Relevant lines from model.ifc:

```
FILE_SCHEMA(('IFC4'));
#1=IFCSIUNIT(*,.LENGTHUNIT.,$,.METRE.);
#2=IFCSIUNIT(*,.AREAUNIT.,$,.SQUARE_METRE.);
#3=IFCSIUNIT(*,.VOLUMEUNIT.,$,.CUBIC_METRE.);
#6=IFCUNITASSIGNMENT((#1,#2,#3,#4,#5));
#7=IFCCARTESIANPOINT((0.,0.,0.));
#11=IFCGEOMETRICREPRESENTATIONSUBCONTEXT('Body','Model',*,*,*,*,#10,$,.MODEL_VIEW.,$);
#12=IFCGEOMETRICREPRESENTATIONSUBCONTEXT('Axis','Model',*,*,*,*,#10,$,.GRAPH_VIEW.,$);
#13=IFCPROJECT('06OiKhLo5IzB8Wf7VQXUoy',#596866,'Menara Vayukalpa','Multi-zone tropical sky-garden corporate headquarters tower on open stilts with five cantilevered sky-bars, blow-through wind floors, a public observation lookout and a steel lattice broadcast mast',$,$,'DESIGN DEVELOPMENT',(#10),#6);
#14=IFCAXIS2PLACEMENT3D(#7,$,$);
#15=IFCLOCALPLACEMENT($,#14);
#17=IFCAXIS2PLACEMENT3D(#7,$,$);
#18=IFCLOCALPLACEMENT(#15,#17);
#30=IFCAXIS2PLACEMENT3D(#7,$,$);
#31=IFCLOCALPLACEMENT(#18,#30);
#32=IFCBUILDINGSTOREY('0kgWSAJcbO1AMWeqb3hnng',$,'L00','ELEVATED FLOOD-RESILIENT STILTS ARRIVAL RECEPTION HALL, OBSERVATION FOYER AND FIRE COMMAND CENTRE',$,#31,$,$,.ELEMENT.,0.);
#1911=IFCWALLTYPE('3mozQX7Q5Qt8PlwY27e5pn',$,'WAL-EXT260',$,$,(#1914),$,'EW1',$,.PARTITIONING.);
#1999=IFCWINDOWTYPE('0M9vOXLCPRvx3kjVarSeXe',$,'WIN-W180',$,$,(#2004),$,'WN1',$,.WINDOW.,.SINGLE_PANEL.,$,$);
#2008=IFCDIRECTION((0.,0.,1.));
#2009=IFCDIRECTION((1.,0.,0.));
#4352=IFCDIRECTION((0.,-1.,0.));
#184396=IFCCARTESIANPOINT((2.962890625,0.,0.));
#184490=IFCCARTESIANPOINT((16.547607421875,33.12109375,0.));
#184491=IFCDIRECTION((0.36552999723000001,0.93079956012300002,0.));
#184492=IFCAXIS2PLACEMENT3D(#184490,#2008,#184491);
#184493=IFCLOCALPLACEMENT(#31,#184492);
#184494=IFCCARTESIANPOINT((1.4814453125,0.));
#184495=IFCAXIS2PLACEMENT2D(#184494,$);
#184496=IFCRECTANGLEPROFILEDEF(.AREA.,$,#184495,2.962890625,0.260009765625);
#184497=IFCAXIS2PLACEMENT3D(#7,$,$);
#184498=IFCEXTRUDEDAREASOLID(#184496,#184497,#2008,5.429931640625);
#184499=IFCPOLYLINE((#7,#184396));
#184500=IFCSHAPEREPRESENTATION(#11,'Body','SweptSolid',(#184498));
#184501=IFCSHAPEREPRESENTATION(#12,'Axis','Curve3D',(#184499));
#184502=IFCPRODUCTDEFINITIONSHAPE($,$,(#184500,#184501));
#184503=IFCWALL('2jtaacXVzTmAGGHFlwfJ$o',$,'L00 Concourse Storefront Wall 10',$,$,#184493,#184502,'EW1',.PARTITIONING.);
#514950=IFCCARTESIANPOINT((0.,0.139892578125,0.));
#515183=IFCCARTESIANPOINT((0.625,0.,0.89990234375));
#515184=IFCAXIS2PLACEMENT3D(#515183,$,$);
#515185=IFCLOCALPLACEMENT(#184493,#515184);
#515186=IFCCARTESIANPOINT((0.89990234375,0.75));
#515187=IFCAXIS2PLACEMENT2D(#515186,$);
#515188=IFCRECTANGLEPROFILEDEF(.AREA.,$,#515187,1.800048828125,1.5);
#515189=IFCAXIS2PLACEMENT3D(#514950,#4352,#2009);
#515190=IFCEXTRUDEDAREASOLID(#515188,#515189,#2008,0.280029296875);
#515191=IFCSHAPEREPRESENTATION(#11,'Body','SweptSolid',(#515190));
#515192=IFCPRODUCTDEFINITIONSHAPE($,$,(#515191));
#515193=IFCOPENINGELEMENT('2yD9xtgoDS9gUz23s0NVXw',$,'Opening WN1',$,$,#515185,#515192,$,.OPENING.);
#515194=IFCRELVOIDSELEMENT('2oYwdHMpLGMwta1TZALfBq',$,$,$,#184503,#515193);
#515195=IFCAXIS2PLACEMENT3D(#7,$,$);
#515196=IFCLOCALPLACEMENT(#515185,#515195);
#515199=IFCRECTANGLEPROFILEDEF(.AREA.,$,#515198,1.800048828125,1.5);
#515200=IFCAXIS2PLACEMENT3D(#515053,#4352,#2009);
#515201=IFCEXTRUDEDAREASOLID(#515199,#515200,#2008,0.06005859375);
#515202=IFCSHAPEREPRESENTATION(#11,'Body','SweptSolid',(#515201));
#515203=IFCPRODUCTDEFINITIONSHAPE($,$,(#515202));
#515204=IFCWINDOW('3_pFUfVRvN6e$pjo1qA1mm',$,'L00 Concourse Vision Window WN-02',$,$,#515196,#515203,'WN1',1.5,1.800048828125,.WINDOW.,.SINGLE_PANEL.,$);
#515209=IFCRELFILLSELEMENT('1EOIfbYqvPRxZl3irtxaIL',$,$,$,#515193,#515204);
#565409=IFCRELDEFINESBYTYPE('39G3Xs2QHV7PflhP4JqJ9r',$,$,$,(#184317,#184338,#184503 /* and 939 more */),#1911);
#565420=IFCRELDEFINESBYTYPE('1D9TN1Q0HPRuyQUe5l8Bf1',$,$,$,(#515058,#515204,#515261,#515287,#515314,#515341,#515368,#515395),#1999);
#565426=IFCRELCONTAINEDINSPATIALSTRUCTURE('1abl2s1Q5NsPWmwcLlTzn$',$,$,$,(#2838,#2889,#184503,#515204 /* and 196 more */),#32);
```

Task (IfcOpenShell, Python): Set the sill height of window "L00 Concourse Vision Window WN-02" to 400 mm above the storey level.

```python
import numpy as np
import ifcopenshell
import ifcopenshell.api.geometry
import ifcopenshell.geom
import ifcopenshell.util.element
import ifcopenshell.util.placement
import ifcopenshell.util.shape
import ifcopenshell.util.unit

model = ifcopenshell.open("model.ifc")
unit_scale = ifcopenshell.util.unit.calculate_unit_scale(model)

window = model.by_id(515204)
opening = window.FillsVoids[0].RelatingOpeningElement
storey = ifcopenshell.util.element.get_container(window, ifc_class="IfcBuildingStorey")
level = ifcopenshell.util.placement.get_local_placement(storey.ObjectPlacement)[2, 3]

# The opening's origin need not be at the sill, so measure its lowest point.
shape = ifcopenshell.geom.create_shape(ifcopenshell.geom.settings(), opening)
bottom = ifcopenshell.util.shape.get_shape_bottom_elevation(shape, shape.geometry) / unit_scale
dz = level + 0.4 / unit_scale - bottom

shift = np.array([0.0, 0.0, dz])
# The window is placed relative to its opening, so it follows when the opening moves.
matrix = ifcopenshell.util.placement.get_local_placement(opening.ObjectPlacement)
matrix[:3, 3] += shift
ifcopenshell.api.geometry.edit_object_placement(
    model, product=opening, matrix=matrix, is_si=False, should_transform_children=True
)

print(f"moved by {dz * unit_scale:+.3f} m")

model.write("model_updated.ifc")
```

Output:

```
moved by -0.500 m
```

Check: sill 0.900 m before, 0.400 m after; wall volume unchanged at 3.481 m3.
